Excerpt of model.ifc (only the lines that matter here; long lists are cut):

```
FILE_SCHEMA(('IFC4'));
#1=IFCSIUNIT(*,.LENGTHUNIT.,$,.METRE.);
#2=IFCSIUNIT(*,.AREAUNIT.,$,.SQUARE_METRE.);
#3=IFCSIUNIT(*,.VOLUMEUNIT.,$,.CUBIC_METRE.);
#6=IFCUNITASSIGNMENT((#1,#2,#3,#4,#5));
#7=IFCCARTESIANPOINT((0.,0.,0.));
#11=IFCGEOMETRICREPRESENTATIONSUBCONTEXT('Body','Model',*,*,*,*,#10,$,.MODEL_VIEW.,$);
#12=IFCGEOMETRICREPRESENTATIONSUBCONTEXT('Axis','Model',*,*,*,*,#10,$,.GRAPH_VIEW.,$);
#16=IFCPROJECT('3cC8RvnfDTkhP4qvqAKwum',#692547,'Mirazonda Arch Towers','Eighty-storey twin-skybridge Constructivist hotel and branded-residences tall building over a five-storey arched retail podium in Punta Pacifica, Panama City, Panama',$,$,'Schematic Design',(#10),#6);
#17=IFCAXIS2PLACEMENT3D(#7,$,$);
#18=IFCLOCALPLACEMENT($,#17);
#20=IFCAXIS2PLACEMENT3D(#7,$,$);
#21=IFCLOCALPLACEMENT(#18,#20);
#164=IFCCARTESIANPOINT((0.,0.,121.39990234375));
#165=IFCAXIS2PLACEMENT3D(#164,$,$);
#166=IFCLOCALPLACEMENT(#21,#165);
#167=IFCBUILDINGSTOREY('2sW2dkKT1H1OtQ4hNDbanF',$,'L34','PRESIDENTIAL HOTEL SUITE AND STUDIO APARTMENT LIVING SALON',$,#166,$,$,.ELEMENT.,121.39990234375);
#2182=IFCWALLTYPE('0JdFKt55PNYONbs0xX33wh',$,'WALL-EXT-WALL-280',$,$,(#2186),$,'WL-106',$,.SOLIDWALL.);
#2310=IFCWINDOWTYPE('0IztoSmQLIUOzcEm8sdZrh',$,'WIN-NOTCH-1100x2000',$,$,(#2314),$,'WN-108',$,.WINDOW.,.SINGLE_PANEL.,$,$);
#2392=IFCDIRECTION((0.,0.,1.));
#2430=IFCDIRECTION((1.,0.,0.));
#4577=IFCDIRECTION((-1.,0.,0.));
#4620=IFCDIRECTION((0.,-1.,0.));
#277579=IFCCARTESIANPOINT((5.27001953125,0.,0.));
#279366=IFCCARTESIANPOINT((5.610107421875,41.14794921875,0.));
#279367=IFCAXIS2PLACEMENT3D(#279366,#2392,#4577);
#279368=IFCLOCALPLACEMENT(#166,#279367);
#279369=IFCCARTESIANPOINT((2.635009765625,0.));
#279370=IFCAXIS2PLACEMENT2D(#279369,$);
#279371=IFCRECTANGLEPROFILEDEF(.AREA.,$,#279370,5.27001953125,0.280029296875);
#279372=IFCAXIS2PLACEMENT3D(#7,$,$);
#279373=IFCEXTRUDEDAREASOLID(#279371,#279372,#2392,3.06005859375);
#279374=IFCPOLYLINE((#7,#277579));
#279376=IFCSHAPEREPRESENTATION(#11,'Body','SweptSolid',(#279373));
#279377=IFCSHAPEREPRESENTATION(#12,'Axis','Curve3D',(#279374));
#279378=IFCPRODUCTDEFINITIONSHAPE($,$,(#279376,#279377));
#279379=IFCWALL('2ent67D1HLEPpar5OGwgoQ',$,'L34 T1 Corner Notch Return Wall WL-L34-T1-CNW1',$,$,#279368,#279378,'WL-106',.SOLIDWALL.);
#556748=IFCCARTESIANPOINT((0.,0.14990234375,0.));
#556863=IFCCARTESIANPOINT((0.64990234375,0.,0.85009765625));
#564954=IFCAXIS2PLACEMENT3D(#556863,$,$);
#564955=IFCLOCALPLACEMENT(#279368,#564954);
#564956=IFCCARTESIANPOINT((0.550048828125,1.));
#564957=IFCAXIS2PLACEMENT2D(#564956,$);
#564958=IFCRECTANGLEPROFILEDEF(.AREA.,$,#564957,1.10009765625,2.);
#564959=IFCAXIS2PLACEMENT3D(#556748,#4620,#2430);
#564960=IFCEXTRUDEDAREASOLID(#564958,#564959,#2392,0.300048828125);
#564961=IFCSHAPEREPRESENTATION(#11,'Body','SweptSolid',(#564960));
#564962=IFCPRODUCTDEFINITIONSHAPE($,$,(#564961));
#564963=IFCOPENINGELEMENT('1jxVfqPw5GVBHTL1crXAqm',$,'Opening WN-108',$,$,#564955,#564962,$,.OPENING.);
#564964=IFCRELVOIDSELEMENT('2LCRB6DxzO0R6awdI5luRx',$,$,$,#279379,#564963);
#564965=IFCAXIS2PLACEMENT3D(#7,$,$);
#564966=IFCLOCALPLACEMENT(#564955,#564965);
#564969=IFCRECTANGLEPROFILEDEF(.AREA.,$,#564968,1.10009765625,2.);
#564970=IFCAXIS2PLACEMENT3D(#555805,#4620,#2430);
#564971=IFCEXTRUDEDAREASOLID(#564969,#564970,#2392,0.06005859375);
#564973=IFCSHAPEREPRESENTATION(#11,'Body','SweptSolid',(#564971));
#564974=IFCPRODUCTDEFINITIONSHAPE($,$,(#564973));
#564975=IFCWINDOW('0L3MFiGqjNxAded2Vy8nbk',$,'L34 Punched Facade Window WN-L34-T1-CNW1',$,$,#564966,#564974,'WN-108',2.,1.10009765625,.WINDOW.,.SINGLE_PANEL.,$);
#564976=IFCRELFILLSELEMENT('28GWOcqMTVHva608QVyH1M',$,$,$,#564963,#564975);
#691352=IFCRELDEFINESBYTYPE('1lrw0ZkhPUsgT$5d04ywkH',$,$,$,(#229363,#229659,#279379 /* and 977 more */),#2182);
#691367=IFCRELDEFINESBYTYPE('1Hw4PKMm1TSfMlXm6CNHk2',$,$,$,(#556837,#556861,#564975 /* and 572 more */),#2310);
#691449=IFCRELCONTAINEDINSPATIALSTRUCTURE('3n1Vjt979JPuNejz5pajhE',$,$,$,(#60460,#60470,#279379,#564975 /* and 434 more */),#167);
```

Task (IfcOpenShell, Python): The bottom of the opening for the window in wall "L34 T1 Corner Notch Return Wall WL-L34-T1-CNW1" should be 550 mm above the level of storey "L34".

```python
import numpy as np
import ifcopenshell
import ifcopenshell.api.geometry
import ifcopenshell.geom
import ifcopenshell.util.element
import ifcopenshell.util.placement
import ifcopenshell.util.shape
import ifcopenshell.util.unit

model = ifcopenshell.open("model.ifc")
unit_scale = ifcopenshell.util.unit.calculate_unit_scale(model)

window = model.by_guid("0L3MFiGqjNxAded2Vy8nbk")
opening = window.FillsVoids[0].RelatingOpeningElement
storey = ifcopenshell.util.element.get_container(window, ifc_class="IfcBuildingStorey")
level = ifcopenshell.util.placement.get_local_placement(storey.ObjectPlacement)[2, 3]

# The opening's origin need not be at the sill, so measure its lowest point.
shape = ifcopenshell.geom.create_shape(ifcopenshell.geom.settings(), opening)
bottom = ifcopenshell.util.shape.get_shape_bottom_elevation(shape, shape.geometry) / unit_scale
dz = level + 0.55 / unit_scale - bottom

shift = np.array([0.0, 0.0, dz])
# The window is placed relative to its opening, so it follows when the opening moves.
matrix = ifcopenshell.util.placement.get_local_placement(opening.ObjectPlacement)
matrix[:3, 3] += shift
ifcopenshell.api.geometry.edit_object_placement(
    model, product=opening, matrix=matrix, is_si=False, should_transform_children=True
)

print(f"moved by {dz * unit_scale:+.3f} m")

model.write("model_updated.ifc")
```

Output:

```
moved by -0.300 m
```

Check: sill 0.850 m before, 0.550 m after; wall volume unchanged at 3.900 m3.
